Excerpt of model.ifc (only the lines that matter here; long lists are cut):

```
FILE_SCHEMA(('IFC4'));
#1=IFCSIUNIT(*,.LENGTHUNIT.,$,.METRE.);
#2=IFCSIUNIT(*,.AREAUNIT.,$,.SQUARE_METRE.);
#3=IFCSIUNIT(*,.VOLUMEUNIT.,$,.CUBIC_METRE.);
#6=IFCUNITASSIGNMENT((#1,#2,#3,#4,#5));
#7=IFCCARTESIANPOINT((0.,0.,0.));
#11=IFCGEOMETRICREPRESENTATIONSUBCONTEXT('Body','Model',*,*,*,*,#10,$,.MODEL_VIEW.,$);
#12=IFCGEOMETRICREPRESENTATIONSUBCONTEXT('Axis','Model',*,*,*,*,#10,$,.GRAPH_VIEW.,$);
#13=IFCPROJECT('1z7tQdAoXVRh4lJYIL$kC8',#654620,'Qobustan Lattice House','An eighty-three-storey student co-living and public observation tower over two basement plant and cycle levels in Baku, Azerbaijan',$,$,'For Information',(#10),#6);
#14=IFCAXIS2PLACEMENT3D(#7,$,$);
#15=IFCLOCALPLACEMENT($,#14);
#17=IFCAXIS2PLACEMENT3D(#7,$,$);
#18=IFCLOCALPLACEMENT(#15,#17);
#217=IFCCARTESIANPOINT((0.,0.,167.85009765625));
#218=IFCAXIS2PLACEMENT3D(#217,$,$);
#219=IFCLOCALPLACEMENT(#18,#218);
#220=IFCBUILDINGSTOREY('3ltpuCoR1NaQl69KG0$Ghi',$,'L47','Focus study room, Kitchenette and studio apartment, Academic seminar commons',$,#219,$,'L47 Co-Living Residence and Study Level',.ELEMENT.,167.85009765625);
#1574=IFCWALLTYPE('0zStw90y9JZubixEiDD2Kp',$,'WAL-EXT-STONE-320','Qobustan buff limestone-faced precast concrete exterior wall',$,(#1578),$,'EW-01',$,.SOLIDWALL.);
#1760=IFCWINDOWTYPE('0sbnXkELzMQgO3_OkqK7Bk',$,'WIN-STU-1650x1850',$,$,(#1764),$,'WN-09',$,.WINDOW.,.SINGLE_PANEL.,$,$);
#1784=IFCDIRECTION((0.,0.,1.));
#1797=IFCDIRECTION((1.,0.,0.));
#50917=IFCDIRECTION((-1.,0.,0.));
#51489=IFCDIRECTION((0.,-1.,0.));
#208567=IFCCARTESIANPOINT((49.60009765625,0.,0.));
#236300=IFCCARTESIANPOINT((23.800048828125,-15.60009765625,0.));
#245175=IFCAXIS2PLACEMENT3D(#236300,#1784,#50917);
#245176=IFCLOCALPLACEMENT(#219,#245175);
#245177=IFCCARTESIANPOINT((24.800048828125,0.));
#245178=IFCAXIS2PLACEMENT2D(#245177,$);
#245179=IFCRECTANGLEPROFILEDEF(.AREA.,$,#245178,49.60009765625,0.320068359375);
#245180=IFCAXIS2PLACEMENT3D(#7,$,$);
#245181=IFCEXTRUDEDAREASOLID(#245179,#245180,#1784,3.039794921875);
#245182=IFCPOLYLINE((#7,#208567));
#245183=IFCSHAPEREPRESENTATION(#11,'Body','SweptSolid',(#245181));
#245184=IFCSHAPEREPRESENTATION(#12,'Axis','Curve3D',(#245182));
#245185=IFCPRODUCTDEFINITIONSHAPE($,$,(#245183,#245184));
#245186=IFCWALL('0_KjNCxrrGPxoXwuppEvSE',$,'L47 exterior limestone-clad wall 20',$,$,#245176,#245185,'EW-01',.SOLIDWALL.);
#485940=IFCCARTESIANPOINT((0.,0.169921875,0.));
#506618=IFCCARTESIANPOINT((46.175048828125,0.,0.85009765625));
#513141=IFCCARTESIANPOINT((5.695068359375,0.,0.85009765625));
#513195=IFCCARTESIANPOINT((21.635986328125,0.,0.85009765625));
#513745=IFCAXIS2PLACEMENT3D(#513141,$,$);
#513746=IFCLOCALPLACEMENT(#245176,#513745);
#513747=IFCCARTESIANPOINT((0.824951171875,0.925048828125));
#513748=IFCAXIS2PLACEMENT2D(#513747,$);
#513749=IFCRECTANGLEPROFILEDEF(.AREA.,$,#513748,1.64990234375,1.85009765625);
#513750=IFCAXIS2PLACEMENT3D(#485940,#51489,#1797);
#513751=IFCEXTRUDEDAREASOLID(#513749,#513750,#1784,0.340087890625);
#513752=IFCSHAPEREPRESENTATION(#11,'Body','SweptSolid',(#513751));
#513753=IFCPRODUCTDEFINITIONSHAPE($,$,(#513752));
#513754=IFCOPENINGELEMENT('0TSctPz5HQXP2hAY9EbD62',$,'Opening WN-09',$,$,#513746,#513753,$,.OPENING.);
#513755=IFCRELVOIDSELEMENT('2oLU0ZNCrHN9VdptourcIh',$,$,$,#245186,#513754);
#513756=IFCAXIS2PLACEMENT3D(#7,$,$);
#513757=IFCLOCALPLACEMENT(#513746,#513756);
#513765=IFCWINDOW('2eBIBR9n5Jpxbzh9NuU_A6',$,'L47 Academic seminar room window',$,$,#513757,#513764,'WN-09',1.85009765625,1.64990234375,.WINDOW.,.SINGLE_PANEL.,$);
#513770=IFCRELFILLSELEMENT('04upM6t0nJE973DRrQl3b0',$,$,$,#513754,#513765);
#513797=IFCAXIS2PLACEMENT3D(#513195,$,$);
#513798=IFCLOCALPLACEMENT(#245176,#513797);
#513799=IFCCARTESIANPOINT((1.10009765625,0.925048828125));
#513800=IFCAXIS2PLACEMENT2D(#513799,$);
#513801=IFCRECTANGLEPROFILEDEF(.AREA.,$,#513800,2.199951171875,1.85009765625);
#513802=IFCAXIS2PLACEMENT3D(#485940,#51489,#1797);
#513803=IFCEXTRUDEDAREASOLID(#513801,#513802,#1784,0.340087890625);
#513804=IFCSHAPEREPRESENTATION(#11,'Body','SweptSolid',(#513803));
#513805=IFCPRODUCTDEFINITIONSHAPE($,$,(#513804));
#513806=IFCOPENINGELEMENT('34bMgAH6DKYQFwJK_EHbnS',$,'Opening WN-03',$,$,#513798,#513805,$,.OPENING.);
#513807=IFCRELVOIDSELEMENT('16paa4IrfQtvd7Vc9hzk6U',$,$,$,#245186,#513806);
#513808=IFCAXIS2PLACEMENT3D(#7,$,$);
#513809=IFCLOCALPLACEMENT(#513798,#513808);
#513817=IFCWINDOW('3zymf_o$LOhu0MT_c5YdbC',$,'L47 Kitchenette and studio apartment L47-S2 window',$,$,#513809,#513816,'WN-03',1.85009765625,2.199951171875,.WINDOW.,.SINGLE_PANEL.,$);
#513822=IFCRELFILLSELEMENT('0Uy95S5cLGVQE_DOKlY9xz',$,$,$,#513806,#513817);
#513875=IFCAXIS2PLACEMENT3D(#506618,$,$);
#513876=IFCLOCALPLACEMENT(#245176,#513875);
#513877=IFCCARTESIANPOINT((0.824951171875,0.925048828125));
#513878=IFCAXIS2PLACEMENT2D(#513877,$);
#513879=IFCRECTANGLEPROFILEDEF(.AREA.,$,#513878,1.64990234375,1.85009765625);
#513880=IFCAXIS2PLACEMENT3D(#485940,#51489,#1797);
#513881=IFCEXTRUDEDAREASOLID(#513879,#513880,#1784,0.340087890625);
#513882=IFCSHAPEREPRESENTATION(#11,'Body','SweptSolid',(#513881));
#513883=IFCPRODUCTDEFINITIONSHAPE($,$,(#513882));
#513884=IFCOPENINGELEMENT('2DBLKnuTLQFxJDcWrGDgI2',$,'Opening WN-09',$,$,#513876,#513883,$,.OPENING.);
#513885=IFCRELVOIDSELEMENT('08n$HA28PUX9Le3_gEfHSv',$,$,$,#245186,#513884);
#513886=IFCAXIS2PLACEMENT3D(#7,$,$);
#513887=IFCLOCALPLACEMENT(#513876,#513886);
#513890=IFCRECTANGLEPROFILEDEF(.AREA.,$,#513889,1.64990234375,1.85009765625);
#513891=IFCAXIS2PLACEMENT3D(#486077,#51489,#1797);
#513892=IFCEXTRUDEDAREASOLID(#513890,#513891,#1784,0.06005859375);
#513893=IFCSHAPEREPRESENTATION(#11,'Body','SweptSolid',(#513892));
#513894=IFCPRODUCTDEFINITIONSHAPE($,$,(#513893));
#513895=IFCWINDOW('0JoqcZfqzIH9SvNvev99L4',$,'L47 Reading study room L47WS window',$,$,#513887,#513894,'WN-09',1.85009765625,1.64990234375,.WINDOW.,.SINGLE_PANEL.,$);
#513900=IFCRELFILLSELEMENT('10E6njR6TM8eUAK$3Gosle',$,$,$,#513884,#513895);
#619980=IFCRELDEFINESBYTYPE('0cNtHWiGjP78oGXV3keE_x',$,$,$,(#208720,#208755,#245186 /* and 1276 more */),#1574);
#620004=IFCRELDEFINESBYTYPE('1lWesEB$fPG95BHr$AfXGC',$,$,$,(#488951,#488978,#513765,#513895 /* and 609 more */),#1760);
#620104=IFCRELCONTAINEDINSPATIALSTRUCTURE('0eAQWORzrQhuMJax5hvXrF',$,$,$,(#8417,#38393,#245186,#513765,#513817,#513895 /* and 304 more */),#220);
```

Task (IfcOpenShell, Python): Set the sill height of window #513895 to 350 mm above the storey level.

```python
import numpy as np
import ifcopenshell
import ifcopenshell.api.geometry
import ifcopenshell.geom
import ifcopenshell.util.element
import ifcopenshell.util.placement
import ifcopenshell.util.shape
import ifcopenshell.util.unit

model = ifcopenshell.open("model.ifc")
unit_scale = ifcopenshell.util.unit.calculate_unit_scale(model)

window = model.by_guid("0JoqcZfqzIH9SvNvev99L4")
opening = window.FillsVoids[0].RelatingOpeningElement
storey = ifcopenshell.util.element.get_container(window, ifc_class="IfcBuildingStorey")
level = ifcopenshell.util.placement.get_local_placement(storey.ObjectPlacement)[2, 3]

# The opening's origin need not be at the sill, so measure its lowest point.
shape = ifcopenshell.geom.create_shape(ifcopenshell.geom.settings(), opening)
bottom = ifcopenshell.util.shape.get_shape_bottom_elevation(shape, shape.geometry) / unit_scale
dz = level + 0.35 / unit_scale - bottom

shift = np.array([0.0, 0.0, dz])
# The window is placed relative to its opening, so it follows when the opening moves.
matrix = ifcopenshell.util.placement.get_local_placement(opening.ObjectPlacement)
matrix[:3, 3] += shift
ifcopenshell.api.geometry.edit_object_placement(
    model, product=opening, matrix=matrix, is_si=False, should_transform_children=True
)

print(f"moved by {dz * unit_scale:+.3f} m")

model.write("model_v2.ifc")
```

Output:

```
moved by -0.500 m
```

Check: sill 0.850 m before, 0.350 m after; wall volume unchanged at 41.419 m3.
